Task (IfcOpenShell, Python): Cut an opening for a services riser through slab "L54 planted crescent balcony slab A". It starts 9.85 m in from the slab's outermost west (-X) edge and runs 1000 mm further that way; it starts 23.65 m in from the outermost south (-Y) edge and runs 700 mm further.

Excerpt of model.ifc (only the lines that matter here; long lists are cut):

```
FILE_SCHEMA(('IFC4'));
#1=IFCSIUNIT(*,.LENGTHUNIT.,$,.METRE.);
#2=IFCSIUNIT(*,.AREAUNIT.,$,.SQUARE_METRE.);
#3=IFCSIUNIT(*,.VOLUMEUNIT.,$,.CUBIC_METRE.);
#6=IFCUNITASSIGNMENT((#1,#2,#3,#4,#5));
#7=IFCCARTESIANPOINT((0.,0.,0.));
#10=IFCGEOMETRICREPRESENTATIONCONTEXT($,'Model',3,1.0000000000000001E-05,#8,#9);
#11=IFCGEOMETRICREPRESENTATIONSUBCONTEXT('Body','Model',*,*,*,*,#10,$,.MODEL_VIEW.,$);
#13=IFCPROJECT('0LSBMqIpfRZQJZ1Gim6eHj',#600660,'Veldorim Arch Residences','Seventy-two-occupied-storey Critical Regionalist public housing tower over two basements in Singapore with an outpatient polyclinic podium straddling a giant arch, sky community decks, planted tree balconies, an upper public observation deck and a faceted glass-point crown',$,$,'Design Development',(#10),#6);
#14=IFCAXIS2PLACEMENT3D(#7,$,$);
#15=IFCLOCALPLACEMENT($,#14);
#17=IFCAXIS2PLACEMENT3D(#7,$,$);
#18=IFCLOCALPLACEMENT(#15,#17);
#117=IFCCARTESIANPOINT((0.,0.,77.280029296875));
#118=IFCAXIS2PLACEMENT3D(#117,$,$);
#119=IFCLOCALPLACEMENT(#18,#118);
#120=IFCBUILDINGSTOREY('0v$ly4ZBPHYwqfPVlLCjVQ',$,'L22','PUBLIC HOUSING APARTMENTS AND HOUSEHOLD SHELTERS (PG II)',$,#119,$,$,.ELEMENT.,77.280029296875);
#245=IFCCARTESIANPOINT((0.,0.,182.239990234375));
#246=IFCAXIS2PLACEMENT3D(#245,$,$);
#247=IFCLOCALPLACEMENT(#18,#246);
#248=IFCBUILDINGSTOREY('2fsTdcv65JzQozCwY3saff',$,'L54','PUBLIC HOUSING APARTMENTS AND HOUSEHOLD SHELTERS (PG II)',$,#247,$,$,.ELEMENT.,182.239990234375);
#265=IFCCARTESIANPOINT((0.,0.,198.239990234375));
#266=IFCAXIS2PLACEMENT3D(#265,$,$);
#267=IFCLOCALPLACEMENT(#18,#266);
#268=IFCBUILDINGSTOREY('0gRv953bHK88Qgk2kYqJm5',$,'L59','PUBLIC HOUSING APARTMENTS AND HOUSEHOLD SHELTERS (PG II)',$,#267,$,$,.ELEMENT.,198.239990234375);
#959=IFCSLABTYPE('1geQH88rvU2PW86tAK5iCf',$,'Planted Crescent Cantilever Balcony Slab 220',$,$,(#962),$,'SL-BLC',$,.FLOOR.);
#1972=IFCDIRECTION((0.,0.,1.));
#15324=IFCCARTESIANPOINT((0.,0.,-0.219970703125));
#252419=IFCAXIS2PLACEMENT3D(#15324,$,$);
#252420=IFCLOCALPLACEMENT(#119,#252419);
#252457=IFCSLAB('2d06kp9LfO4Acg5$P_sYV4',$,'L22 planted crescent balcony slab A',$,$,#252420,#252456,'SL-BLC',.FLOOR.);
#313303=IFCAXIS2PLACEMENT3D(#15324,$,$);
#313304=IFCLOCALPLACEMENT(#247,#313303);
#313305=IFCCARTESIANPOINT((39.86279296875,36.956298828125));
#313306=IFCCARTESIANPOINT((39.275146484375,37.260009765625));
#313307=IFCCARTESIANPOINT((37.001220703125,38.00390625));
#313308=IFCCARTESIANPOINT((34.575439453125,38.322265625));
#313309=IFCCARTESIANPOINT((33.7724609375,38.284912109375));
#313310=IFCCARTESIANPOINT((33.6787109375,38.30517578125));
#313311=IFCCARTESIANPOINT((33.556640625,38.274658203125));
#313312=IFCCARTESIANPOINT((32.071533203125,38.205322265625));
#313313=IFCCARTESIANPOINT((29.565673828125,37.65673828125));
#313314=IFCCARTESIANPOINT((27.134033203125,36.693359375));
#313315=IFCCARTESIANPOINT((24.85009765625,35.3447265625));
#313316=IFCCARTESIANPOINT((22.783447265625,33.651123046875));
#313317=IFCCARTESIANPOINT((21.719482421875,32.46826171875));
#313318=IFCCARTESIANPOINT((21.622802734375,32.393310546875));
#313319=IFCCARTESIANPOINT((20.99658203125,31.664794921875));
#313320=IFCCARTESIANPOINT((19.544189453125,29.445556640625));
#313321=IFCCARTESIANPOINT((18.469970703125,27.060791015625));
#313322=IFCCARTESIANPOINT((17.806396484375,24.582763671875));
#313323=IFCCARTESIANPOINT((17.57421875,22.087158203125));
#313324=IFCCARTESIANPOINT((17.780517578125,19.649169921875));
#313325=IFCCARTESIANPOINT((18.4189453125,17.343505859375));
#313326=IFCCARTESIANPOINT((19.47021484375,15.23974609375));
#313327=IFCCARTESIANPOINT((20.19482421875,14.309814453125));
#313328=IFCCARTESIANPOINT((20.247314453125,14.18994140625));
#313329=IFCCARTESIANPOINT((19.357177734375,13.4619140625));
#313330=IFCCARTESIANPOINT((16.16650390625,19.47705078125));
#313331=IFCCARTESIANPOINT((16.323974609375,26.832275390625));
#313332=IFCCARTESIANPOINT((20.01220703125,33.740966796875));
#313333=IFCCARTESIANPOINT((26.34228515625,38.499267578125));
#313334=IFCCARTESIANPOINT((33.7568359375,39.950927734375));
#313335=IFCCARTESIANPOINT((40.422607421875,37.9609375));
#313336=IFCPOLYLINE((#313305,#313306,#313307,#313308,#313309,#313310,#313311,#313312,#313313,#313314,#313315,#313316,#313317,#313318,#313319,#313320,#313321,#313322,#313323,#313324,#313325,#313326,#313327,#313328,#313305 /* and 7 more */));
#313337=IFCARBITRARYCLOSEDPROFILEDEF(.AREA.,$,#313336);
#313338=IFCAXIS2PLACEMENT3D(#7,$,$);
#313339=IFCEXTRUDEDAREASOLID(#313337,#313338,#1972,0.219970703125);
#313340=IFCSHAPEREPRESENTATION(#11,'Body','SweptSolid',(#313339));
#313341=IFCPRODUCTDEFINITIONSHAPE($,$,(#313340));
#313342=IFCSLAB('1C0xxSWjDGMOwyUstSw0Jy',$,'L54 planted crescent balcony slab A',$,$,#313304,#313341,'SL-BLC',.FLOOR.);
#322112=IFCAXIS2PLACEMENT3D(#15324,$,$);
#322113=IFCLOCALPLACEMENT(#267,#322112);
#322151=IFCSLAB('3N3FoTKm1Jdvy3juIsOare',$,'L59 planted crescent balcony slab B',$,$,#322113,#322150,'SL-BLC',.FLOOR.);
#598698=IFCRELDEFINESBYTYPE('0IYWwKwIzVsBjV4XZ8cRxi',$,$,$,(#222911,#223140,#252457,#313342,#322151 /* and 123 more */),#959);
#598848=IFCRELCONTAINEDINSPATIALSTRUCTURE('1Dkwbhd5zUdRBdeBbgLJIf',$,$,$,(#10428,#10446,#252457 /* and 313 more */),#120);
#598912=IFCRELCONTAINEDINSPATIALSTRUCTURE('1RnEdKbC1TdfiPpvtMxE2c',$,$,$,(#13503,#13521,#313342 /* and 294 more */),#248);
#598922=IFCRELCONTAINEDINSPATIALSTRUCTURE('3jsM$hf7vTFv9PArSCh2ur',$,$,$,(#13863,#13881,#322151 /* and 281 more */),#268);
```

```python
import numpy as np
import ifcopenshell
import ifcopenshell.api.feature
import ifcopenshell.api.geometry
import ifcopenshell.api.root
import ifcopenshell.geom
import ifcopenshell.util.placement
import ifcopenshell.util.representation
import ifcopenshell.util.shape
import ifcopenshell.util.unit

model = ifcopenshell.open("model.ifc")
unit_scale = ifcopenshell.util.unit.calculate_unit_scale(model)
settings = ifcopenshell.geom.settings()


def volume(element):
    """Net volume in cubic metres, openings subtracted."""
    shape = ifcopenshell.geom.create_shape(settings, element)
    return ifcopenshell.util.shape.get_volume(shape.geometry)


slab = model.by_id(313342)
before = volume(slab)

# Extent in the slab's own axes, in metres. The edges named are its -X and -Y sides.
slab_shape = ifcopenshell.geom.create_shape(settings, slab)
vertices = ifcopenshell.util.shape.get_vertices(slab_shape.geometry)
x_min, y_min, bottom = vertices.min(axis=0)
top = vertices[:, 2].max()

opening = ifcopenshell.api.root.create_entity(model, ifc_class="IfcOpeningElement", name="Services riser opening", predefined_type="OPENING")
context = ifcopenshell.util.representation.get_context(model, "Model", "Body", "MODEL_VIEW")
width, depth = 1, 0.7
outline = [(0.0, 0.0), (width, 0.0), (width, depth), (0.0, depth), (0.0, 0.0)]
# Overshoot both faces by 50 mm so the cut is clean.
shape = ifcopenshell.api.geometry.add_slab_representation(
    model, context=context, depth=top - bottom + 0.1, polyline=outline
)
ifcopenshell.api.geometry.assign_representation(model, product=opening, representation=shape)

matrix = ifcopenshell.util.placement.get_local_placement(slab.ObjectPlacement)
matrix[:, 3] = matrix @ np.append(np.array([x_min + 9.85, y_min + 23.65, bottom - 0.05]) / unit_scale, 1.0)
ifcopenshell.api.geometry.edit_object_placement(model, product=opening, matrix=matrix, is_si=False)
ifcopenshell.api.feature.add_feature(model, feature=opening, element=slab)

after = volume(slab)

print(f"slab volume {before:.3f} -> {after:.3f} m3")

model.write("model_edited.ifc")
```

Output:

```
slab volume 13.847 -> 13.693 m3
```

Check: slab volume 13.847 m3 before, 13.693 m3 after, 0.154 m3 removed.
